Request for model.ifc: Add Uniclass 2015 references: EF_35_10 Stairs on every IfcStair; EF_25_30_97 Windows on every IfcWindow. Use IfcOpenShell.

First a look at what the model holds.

```python
import ifcopenshell

model = ifcopenshell.open("model.ifc")
print(model.schema)
print("classifications:", [c.Name for c in model.by_type("IfcClassification")])
for ifc_class in ("IfcDoor", "IfcRoof", "IfcStair", "IfcWall", "IfcWindow"):
    print(ifc_class, len(model.by_type(ifc_class)))
```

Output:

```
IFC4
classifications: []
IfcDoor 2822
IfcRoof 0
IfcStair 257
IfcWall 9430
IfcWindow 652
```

```python
import ifcopenshell
import ifcopenshell.api.classification

model = ifcopenshell.open("model.ifc")

system = ifcopenshell.api.classification.add_classification(model, classification="Uniclass 2015")

codes = {
    "IfcStair": ("EF_35_10", "Stairs"),
    "IfcWindow": ("EF_25_30_97", "Windows"),
}
for ifc_class, (code, name) in codes.items():
    products = model.by_type(ifc_class)
    ifcopenshell.api.classification.add_reference(
        model, products=products, classification=system, identification=code, name=name
    )
    print(code, len(products))

model.write("model-out.ifc")
```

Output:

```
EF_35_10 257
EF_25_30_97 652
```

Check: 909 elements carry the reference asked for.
